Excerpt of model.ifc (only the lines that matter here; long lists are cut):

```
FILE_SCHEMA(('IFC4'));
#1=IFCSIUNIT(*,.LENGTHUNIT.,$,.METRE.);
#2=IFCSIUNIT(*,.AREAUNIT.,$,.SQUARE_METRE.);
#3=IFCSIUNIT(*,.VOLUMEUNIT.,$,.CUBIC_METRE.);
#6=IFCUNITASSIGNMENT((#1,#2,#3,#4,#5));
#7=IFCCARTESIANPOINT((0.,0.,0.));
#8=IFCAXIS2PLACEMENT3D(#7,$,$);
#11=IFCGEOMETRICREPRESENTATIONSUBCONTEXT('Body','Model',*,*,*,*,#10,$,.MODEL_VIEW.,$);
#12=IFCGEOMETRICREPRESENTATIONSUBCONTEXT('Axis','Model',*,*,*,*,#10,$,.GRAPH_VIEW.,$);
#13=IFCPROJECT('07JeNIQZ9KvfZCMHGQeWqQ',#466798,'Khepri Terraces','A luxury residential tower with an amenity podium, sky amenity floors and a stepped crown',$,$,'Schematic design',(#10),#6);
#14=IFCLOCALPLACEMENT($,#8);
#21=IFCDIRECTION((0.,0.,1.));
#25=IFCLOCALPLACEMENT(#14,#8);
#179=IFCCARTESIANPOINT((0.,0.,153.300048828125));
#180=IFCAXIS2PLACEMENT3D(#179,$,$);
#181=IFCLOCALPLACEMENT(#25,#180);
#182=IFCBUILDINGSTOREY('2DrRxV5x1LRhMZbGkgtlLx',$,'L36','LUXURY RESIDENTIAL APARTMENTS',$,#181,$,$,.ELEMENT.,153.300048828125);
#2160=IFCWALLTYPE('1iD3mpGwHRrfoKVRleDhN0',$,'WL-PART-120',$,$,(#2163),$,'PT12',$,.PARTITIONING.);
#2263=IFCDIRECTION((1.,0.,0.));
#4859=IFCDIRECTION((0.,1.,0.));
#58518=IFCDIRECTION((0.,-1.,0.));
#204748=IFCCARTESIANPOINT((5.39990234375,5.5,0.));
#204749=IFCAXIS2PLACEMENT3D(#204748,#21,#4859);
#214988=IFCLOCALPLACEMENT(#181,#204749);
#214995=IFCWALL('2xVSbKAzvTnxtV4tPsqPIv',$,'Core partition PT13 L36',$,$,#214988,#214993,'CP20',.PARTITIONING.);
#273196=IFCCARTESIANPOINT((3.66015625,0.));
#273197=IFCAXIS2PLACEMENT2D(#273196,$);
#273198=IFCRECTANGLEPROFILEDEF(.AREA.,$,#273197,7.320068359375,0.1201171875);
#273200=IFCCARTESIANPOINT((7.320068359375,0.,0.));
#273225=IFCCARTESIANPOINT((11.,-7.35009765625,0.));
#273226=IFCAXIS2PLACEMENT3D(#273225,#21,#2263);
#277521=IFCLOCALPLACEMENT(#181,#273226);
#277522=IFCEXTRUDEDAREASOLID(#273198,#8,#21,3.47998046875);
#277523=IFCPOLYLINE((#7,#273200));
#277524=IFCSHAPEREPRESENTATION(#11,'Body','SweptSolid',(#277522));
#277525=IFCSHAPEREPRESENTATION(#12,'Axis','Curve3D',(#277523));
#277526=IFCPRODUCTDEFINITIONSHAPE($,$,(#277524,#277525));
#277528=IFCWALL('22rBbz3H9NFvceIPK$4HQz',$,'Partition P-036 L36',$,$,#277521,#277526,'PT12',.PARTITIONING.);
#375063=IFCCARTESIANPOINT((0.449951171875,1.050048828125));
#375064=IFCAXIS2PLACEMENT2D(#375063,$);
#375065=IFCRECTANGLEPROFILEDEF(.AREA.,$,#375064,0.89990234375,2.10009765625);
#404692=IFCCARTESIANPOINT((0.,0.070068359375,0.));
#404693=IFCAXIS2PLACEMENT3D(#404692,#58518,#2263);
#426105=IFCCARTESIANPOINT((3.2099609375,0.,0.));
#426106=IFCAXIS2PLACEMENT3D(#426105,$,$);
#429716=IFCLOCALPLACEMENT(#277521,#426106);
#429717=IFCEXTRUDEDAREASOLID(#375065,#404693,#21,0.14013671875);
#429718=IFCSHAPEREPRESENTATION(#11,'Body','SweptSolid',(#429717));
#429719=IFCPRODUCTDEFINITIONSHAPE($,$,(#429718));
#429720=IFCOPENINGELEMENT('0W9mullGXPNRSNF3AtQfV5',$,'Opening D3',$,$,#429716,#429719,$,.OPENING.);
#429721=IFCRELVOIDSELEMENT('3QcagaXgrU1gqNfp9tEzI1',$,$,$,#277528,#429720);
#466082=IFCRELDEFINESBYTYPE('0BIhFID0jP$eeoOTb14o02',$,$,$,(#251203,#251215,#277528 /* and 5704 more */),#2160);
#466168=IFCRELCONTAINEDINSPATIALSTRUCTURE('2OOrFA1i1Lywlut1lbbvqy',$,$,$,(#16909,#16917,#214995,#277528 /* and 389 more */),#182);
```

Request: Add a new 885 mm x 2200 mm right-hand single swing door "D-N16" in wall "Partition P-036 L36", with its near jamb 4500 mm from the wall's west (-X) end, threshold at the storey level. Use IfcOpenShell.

```python
import numpy as np
import ifcopenshell
import ifcopenshell.api.feature
import ifcopenshell.api.geometry
import ifcopenshell.api.root
import ifcopenshell.api.spatial
import ifcopenshell.geom
import ifcopenshell.util.element
import ifcopenshell.util.placement
import ifcopenshell.util.representation
import ifcopenshell.util.shape
import ifcopenshell.util.unit

model = ifcopenshell.open("model.ifc")
unit_scale = ifcopenshell.util.unit.calculate_unit_scale(model)
settings = ifcopenshell.geom.settings()


def volume(element):
    """Net volume in cubic metres, openings subtracted."""
    shape = ifcopenshell.geom.create_shape(settings, element)
    return ifcopenshell.util.shape.get_volume(shape.geometry)


wall = model.by_guid("22rBbz3H9NFvceIPK$4HQz")
storey = ifcopenshell.util.element.get_container(wall, ifc_class="IfcBuildingStorey")
context = ifcopenshell.util.representation.get_context(model, "Model", "Body", "MODEL_VIEW")
before = volume(wall)

width, height, from_end, sill = 0.885, 2.2, 4.5, 0.0  # metres

# The wall runs along its own X axis, and the end named is its -X end.
wall_shape = ifcopenshell.geom.create_shape(settings, wall)
x, y, z = ifcopenshell.util.shape.get_vertices(wall_shape.geometry).T
start = x.min() + from_end
face, thickness = float(y.min()), float(y.max() - y.min())
wall_matrix = ifcopenshell.util.placement.get_local_placement(wall.ObjectPlacement)
level = ifcopenshell.util.placement.get_local_placement(storey.ObjectPlacement)[2, 3]


def in_wall(x, y):
    """Placement at x, y metres in the wall's axes, at sill height."""
    matrix = wall_matrix.copy()
    matrix[:, 3] = wall_matrix @ np.array([x / unit_scale, y / unit_scale, 0.0, 1.0])
    matrix[2, 3] = level + sill / unit_scale
    return matrix


# Opening: a box that overshoots both wall faces by 50 mm.
opening = ifcopenshell.api.root.create_entity(model, ifc_class="IfcOpeningElement", predefined_type="OPENING")
box = ifcopenshell.api.geometry.add_wall_representation(
    model, context=context, length=width, height=height, thickness=thickness + 0.1
)
ifcopenshell.api.geometry.assign_representation(model, product=opening, representation=box)
ifcopenshell.api.geometry.edit_object_placement(model, product=opening, matrix=in_wall(start, face - 0.05), is_si=False)
ifcopenshell.api.feature.add_feature(model, feature=opening, element=wall)

door = ifcopenshell.api.root.create_entity(model, ifc_class="IfcDoor", name="D-N16", predefined_type="DOOR")
door.OverallWidth, door.OverallHeight = width / unit_scale, height / unit_scale
door.OperationType = "SINGLE_SWING_RIGHT"
body = ifcopenshell.api.geometry.add_door_representation(
    model,
    context=context,
    overall_width=door.OverallWidth,
    overall_height=door.OverallHeight,
    operation_type="SINGLE_SWING_RIGHT",
    lining_properties={"LiningDepth": thickness / unit_scale, "ThresholdDepth": thickness / unit_scale},
)
ifcopenshell.api.geometry.assign_representation(model, product=door, representation=body)
ifcopenshell.api.spatial.assign_container(model, products=[door], relating_structure=storey)
ifcopenshell.api.feature.add_filling(model, opening=opening, element=door)

# The lining spans the wall, so the door starts at the wall face.
ifcopenshell.api.geometry.edit_object_placement(model, product=door, matrix=in_wall(start, face), is_si=False)

after = volume(wall)

print(f"wall volume {before:.3f} -> {after:.3f} m3")

model.write("model_updated.ifc")
```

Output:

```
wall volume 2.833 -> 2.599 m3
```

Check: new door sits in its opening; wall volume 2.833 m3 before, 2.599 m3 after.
